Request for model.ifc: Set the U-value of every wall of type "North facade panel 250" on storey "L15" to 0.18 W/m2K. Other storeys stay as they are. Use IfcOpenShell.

First a look at what the model holds.

```python
import ifcopenshell
import ifcopenshell.util.element

model = ifcopenshell.open("model.ifc")
print(model.schema)
storey = next(s for s in model.by_type("IfcBuildingStorey") if s.Name == "L15")
walls = [e for e in ifcopenshell.util.element.get_decomposition(storey) if e.is_a("IfcWall")]
seen = {}
for e in walls:
    element_type = ifcopenshell.util.element.get_type(e)
    key = (element_type.Name if element_type != e and element_type else None, ifcopenshell.util.element.get_pset(e, "Pset_WallCommon", "ThermalTransmittance"))
    seen[key] = seen.get(key, 0) + 1
for (name, value), count in sorted(seen.items(), key=str):
    print(count, "x", name, "|", value)
```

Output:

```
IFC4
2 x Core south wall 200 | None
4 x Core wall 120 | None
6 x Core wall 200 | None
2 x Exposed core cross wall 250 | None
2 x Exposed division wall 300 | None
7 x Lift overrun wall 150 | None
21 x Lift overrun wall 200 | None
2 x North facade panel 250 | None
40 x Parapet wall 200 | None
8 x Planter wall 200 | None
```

```python
import ifcopenshell
import ifcopenshell.api.pset
import ifcopenshell.util.element

model = ifcopenshell.open("model.ifc")

storey = next(s for s in model.by_type("IfcBuildingStorey") if s.Name == "L15")
walls = [e for e in ifcopenshell.util.element.get_decomposition(storey) if e.is_a("IfcWall")]

count = 0
for e in walls:
    element_type = ifcopenshell.util.element.get_type(e)
    if element_type in (None, e) or element_type.Name != "North facade panel 250":
        continue
    # add_pset returns the element's existing set when there is one.
    pset = ifcopenshell.api.pset.add_pset(model, product=e, name="Pset_WallCommon")
    ifcopenshell.api.pset.edit_pset(model, pset=pset, properties={"ThermalTransmittance": 0.18})
    count += 1

print(count, "walls updated")

model.write("model-out.ifc")
```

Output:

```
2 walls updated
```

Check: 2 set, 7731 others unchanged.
